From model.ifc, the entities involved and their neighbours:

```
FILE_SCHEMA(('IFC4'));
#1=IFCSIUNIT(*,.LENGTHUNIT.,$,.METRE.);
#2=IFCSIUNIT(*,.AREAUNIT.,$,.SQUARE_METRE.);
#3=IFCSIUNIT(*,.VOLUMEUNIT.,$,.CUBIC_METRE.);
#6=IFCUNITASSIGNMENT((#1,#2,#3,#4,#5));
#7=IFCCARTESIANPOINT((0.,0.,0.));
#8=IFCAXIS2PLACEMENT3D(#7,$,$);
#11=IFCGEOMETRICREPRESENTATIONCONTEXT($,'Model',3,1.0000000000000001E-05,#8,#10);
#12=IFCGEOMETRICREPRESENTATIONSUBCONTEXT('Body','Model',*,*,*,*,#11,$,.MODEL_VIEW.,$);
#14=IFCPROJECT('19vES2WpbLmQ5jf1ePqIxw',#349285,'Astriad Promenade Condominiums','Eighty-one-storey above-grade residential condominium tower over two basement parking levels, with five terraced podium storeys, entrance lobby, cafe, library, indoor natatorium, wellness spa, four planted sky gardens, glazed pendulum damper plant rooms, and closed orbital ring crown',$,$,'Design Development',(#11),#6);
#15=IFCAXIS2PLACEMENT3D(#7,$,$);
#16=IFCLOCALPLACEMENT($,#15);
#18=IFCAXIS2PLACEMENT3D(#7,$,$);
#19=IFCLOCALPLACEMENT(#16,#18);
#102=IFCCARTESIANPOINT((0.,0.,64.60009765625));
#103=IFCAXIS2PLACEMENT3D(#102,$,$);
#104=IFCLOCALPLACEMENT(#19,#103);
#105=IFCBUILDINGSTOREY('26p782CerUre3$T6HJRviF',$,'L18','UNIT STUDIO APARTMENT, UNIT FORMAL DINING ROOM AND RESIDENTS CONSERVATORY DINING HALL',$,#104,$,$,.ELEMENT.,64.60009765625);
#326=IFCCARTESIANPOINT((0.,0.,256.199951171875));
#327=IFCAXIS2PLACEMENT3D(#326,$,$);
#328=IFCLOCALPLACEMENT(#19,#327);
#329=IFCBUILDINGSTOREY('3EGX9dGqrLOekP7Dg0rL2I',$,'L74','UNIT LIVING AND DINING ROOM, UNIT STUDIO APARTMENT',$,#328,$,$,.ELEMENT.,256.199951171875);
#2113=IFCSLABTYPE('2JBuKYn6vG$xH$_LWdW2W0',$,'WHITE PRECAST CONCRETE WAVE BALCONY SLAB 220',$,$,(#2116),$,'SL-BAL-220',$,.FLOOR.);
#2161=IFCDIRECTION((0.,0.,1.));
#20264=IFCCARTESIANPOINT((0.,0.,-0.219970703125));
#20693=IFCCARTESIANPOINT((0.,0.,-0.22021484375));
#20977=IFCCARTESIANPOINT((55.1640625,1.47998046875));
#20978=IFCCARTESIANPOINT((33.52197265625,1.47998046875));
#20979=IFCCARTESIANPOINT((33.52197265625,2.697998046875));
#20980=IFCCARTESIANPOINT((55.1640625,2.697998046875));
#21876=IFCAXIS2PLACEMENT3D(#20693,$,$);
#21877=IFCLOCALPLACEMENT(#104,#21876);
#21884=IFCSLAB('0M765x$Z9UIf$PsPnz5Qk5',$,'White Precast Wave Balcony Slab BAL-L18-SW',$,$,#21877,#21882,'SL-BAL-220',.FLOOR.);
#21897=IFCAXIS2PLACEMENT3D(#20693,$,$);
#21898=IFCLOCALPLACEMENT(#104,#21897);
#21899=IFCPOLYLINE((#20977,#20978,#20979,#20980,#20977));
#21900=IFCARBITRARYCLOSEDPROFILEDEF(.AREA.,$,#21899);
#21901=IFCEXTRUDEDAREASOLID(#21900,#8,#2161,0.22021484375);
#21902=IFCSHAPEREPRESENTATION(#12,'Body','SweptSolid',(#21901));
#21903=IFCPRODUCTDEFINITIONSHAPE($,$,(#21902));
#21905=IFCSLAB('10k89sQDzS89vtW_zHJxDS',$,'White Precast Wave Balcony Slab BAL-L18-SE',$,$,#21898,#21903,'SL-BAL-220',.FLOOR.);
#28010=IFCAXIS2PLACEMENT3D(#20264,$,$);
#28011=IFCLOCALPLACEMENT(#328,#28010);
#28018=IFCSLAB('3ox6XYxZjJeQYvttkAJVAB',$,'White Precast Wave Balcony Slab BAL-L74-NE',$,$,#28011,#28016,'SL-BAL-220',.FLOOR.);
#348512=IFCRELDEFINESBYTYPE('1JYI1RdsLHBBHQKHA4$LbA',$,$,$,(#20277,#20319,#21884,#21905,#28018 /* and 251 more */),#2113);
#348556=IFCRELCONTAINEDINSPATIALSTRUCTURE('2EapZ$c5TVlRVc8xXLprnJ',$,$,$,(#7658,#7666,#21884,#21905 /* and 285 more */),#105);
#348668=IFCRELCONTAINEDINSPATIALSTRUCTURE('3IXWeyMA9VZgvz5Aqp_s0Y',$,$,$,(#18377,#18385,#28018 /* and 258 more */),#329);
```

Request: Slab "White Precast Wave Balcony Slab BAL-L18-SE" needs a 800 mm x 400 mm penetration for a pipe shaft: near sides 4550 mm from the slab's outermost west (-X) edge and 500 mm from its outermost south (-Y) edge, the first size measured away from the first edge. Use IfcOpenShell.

```python
import numpy as np
import ifcopenshell
import ifcopenshell.api.feature
import ifcopenshell.api.geometry
import ifcopenshell.api.root
import ifcopenshell.geom
import ifcopenshell.util.placement
import ifcopenshell.util.representation
import ifcopenshell.util.shape
import ifcopenshell.util.unit

model = ifcopenshell.open("model.ifc")
unit_scale = ifcopenshell.util.unit.calculate_unit_scale(model)
settings = ifcopenshell.geom.settings()


def volume(element):
    """Net volume in cubic metres, openings subtracted."""
    shape = ifcopenshell.geom.create_shape(settings, element)
    return ifcopenshell.util.shape.get_volume(shape.geometry)


slab = model.by_guid("10k89sQDzS89vtW_zHJxDS")
before = volume(slab)

# Extent in the slab's own axes, in metres. The edges named are its -X and -Y sides.
slab_shape = ifcopenshell.geom.create_shape(settings, slab)
vertices = ifcopenshell.util.shape.get_vertices(slab_shape.geometry)
x_min, y_min, bottom = vertices.min(axis=0)
top = vertices[:, 2].max()

opening = ifcopenshell.api.root.create_entity(model, ifc_class="IfcOpeningElement", name="Pipe shaft opening", predefined_type="OPENING")
context = ifcopenshell.util.representation.get_context(model, "Model", "Body", "MODEL_VIEW")
width, depth = 0.8, 0.4
outline = [(0.0, 0.0), (width, 0.0), (width, depth), (0.0, depth), (0.0, 0.0)]
# Overshoot both faces by 50 mm so the cut is clean.
shape = ifcopenshell.api.geometry.add_slab_representation(
    model, context=context, depth=top - bottom + 0.1, polyline=outline
)
ifcopenshell.api.geometry.assign_representation(model, product=opening, representation=shape)

matrix = ifcopenshell.util.placement.get_local_placement(slab.ObjectPlacement)
matrix[:, 3] = matrix @ np.append(np.array([x_min + 4.55, y_min + 0.5, bottom - 0.05]) / unit_scale, 1.0)
ifcopenshell.api.geometry.edit_object_placement(model, product=opening, matrix=matrix, is_si=False)
ifcopenshell.api.feature.add_feature(model, feature=opening, element=slab)

after = volume(slab)

print(f"slab volume {before:.3f} -> {after:.3f} m3")

model.write("model_v2.ifc")
```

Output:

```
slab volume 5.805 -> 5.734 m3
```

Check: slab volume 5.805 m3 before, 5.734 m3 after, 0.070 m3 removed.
